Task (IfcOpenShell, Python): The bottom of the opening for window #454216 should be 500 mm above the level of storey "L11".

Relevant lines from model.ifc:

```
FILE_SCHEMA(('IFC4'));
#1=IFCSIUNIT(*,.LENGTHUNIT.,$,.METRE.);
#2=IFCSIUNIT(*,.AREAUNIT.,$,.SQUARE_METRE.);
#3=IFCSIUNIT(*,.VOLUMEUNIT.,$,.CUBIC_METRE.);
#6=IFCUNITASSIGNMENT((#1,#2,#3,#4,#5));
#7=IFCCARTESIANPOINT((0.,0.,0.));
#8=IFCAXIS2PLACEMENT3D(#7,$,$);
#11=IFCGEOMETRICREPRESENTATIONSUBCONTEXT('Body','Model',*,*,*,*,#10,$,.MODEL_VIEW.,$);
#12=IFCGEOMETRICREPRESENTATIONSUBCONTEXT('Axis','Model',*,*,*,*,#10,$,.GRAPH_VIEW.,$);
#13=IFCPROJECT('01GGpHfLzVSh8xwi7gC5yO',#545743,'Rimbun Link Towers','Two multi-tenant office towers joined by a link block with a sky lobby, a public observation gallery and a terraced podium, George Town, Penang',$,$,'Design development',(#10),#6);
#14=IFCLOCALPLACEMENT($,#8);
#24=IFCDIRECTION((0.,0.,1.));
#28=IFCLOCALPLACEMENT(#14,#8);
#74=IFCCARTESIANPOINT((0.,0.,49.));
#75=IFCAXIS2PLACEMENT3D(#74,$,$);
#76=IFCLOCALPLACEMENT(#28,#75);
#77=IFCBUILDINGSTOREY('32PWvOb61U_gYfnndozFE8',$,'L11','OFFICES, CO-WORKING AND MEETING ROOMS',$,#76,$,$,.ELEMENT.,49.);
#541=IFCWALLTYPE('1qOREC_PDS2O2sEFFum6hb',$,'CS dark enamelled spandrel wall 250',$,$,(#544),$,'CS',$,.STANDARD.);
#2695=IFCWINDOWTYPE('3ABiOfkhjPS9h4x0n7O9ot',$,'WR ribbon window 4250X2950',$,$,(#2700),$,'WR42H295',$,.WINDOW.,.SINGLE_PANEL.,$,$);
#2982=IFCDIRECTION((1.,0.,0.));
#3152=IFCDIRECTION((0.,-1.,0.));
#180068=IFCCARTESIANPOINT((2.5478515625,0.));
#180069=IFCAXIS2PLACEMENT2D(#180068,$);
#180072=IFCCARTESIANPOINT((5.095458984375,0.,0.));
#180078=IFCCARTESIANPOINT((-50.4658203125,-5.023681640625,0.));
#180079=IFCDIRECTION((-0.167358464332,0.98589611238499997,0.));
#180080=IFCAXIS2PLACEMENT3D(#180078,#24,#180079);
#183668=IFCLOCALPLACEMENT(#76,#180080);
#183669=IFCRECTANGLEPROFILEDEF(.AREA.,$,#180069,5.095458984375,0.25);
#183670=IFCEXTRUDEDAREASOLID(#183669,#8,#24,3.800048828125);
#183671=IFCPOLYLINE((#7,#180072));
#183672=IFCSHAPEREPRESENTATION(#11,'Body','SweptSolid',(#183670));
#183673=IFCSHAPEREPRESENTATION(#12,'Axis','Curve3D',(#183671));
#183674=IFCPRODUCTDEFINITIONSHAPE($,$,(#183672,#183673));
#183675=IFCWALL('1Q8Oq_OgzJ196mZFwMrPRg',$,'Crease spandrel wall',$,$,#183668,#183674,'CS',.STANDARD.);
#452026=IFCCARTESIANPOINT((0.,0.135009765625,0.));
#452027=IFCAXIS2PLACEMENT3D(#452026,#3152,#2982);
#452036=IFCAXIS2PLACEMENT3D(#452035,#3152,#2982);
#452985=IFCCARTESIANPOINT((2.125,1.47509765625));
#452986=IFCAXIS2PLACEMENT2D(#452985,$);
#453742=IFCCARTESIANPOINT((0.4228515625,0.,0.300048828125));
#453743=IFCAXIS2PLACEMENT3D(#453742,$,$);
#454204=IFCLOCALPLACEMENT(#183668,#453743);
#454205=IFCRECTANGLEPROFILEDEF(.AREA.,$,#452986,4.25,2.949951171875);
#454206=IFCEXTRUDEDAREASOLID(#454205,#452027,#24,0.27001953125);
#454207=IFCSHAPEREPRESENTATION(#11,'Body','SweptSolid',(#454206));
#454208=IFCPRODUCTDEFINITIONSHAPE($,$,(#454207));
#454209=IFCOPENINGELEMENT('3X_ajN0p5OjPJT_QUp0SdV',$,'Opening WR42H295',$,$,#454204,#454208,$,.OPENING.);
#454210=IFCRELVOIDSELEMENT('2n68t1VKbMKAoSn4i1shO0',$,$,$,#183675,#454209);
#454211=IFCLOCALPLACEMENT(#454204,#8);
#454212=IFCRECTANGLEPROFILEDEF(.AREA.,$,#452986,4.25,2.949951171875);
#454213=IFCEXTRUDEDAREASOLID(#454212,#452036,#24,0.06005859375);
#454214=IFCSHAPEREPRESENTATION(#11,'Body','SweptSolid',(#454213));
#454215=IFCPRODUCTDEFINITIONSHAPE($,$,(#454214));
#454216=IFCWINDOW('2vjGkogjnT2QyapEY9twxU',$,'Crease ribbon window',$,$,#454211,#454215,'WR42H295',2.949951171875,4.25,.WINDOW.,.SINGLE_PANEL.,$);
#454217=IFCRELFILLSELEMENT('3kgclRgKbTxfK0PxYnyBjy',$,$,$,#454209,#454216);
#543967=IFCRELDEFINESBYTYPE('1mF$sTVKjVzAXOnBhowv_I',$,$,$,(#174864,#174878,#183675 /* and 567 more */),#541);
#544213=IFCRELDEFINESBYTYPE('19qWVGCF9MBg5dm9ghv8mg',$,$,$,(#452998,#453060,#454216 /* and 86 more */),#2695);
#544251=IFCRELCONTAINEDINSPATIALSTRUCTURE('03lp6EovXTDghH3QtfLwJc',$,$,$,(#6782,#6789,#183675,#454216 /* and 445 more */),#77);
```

```python
import numpy as np
import ifcopenshell
import ifcopenshell.api.geometry
import ifcopenshell.geom
import ifcopenshell.util.element
import ifcopenshell.util.placement
import ifcopenshell.util.shape
import ifcopenshell.util.unit

model = ifcopenshell.open("model.ifc")
unit_scale = ifcopenshell.util.unit.calculate_unit_scale(model)

window = model.by_guid("2vjGkogjnT2QyapEY9twxU")
opening = window.FillsVoids[0].RelatingOpeningElement
storey = ifcopenshell.util.element.get_container(window, ifc_class="IfcBuildingStorey")
level = ifcopenshell.util.placement.get_local_placement(storey.ObjectPlacement)[2, 3]

# The opening's origin need not be at the sill, so measure its lowest point.
shape = ifcopenshell.geom.create_shape(ifcopenshell.geom.settings(), opening)
bottom = ifcopenshell.util.shape.get_shape_bottom_elevation(shape, shape.geometry) / unit_scale
dz = level + 0.5 - bottom

shift = np.array([0.0, 0.0, dz])
# The window is placed relative to its opening, so it follows when the opening moves.
matrix = ifcopenshell.util.placement.get_local_placement(opening.ObjectPlacement)
matrix[:3, 3] += shift
ifcopenshell.api.geometry.edit_object_placement(
    model, product=opening, matrix=matrix, is_si=False, should_transform_children=True
)

print(f"moved by {dz * unit_scale:+.3f} m")

model.write("model_edited.ifc")
```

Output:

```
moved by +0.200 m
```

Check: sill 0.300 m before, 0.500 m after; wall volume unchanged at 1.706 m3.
